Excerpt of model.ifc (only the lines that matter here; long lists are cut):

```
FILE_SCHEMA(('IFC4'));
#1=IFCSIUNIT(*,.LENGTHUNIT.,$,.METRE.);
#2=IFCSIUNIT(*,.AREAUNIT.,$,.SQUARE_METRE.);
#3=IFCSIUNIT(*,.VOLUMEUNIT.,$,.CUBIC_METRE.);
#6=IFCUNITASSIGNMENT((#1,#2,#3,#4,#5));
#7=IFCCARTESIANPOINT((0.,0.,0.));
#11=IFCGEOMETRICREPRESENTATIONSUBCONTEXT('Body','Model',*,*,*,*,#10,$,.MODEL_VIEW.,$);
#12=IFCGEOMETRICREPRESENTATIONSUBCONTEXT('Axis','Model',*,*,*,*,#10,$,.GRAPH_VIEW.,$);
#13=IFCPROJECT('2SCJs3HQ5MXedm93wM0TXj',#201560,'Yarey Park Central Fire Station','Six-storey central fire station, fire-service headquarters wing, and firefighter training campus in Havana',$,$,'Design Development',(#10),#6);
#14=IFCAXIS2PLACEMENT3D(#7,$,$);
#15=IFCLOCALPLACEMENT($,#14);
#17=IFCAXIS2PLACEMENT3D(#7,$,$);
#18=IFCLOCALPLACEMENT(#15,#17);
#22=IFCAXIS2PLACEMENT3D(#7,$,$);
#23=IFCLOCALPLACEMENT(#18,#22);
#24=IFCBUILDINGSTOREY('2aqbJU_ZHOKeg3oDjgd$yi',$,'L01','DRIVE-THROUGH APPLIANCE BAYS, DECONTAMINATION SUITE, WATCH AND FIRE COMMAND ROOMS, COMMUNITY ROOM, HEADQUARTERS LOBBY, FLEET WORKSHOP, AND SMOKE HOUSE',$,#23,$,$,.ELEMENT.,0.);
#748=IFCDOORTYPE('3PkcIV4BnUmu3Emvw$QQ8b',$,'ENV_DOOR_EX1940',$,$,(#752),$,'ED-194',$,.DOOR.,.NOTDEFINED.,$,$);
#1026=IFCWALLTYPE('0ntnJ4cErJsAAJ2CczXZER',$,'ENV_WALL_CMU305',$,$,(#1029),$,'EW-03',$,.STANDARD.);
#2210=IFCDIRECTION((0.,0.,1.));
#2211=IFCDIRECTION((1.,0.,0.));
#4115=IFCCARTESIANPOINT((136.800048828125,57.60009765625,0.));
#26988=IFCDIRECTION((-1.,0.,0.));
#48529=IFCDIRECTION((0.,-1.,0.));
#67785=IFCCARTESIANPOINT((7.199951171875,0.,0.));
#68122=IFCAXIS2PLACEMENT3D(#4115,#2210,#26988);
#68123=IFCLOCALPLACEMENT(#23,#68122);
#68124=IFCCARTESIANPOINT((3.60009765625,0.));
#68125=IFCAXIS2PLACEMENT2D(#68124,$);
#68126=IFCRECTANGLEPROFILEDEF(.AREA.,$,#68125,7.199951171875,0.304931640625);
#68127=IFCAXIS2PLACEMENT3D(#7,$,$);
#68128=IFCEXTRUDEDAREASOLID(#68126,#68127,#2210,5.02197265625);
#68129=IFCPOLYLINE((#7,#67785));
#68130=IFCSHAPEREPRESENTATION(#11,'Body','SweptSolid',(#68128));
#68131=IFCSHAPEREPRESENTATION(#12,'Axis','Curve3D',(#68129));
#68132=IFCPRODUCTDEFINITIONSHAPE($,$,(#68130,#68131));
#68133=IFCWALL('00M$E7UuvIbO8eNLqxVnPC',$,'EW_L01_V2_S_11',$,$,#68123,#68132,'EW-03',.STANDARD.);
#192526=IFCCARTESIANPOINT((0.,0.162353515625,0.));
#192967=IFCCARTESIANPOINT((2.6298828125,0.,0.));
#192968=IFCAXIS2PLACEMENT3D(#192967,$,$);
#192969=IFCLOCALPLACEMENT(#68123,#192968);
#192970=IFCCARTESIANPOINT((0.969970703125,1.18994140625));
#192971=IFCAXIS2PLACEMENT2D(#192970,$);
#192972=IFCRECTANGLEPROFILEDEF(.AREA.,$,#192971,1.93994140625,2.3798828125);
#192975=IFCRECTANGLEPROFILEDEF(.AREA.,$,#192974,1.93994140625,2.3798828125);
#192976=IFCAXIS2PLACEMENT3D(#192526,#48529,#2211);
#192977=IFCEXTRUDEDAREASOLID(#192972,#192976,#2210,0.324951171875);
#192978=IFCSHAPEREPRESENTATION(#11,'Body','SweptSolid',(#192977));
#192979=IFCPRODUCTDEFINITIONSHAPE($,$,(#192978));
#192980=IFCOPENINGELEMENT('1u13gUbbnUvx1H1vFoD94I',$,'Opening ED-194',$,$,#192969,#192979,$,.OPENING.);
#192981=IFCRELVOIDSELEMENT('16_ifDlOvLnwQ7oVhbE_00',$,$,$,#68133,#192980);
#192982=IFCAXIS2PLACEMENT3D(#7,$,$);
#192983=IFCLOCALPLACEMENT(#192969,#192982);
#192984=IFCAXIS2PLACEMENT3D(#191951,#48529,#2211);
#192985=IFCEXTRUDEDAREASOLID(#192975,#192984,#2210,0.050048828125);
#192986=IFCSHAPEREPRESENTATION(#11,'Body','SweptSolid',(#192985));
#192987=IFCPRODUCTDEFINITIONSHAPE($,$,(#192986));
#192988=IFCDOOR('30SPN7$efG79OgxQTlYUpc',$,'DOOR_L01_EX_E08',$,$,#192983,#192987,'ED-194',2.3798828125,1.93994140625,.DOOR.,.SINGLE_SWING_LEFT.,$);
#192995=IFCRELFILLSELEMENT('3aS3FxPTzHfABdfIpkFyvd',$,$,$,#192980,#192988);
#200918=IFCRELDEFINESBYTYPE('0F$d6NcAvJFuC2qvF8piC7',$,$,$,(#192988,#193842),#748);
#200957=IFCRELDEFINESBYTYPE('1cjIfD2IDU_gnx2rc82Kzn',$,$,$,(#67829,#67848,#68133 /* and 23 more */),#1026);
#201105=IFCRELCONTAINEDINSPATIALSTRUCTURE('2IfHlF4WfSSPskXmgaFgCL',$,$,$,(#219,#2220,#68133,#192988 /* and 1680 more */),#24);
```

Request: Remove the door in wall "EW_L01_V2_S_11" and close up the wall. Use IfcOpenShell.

```python
import ifcopenshell
import ifcopenshell.api.feature
import ifcopenshell.api.root
import ifcopenshell.geom
import ifcopenshell.util.shape

model = ifcopenshell.open("model.ifc")
settings = ifcopenshell.geom.settings()


def volume(element):
    """Net volume in cubic metres, openings subtracted."""
    shape = ifcopenshell.geom.create_shape(settings, element)
    return ifcopenshell.util.shape.get_volume(shape.geometry)


door = model.by_guid("30SPN7$efG79OgxQTlYUpc")
opening = door.FillsVoids[0].RelatingOpeningElement
wall = opening.VoidsElements[0].RelatingBuildingElement
before = volume(wall)

ifcopenshell.api.root.remove_product(model, product=door)
ifcopenshell.api.feature.remove_feature(model, feature=opening)

after = volume(wall)

print(f"wall volume {before:.3f} -> {after:.3f} m3")

model.write("model_updated.ifc")
```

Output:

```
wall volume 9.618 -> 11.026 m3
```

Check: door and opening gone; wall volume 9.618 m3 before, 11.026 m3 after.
